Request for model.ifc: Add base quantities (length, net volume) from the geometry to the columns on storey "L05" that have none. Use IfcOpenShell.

First a look at what the model holds.

```python
import ifcopenshell
import ifcopenshell.util.element
import ifcopenshell.util.unit

model = ifcopenshell.open("model.ifc")
print(model.schema)
for unit_type in ("LENGTHUNIT", "AREAUNIT", "VOLUMEUNIT"):
    print(unit_type, ifcopenshell.util.unit.calculate_unit_scale(model, unit_type))
storey = next(s for s in model.by_type("IfcBuildingStorey") if s.Name == "L05")
columns = [e for e in ifcopenshell.util.element.get_decomposition(storey) if e.is_a("IfcColumn")]
for e in sorted(columns, key=lambda e: e.id()):
    print(e.id(), e.is_a(), e.Name, list(ifcopenshell.util.element.get_psets(e, qtos_only=True)), sep=" | ")
```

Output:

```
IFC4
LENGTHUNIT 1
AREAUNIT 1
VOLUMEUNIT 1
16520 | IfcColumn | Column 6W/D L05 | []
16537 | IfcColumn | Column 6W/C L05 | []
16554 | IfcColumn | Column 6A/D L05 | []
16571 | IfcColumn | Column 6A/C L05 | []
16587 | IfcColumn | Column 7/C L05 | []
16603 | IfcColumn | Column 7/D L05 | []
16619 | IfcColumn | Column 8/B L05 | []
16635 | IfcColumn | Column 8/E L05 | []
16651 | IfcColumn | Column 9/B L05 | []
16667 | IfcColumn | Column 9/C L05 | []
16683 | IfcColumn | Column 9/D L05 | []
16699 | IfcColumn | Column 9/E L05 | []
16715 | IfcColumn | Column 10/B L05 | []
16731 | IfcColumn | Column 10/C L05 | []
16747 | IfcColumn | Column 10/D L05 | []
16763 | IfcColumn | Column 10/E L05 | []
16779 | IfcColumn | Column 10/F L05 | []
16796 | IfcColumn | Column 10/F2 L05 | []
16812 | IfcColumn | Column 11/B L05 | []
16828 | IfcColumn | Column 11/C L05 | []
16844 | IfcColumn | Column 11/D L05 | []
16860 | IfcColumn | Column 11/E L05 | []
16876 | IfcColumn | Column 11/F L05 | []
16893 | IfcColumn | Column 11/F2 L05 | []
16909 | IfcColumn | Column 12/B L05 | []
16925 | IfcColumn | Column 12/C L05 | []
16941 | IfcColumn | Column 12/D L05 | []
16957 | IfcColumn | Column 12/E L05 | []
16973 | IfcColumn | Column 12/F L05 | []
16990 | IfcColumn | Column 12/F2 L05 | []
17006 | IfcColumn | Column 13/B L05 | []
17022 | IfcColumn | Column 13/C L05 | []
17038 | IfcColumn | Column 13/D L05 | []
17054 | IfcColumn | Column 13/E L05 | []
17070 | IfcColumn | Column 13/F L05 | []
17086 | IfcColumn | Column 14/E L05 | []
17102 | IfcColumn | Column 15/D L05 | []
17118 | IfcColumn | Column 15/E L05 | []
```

```python
import ifcopenshell
import ifcopenshell.api.pset
import ifcopenshell.geom
import ifcopenshell.util.element
import ifcopenshell.util.shape
import ifcopenshell.util.unit

model = ifcopenshell.open("model.ifc")
unit_scale = ifcopenshell.util.unit.calculate_unit_scale(model)
volume_scale = ifcopenshell.util.unit.calculate_unit_scale(model, "VOLUMEUNIT")
settings = ifcopenshell.geom.settings()

storey = next(s for s in model.by_type("IfcBuildingStorey") if s.Name == "L05")
columns = [e for e in ifcopenshell.util.element.get_decomposition(storey) if e.is_a("IfcColumn")]

for e in sorted(columns, key=lambda e: e.id()):
    if ifcopenshell.util.element.get_psets(e, qtos_only=True, should_inherit=False):
        continue
    # Geometry comes back in metres, in the element's own axes.
    shape = ifcopenshell.geom.create_shape(settings, e)
    values = {
        "Length": ifcopenshell.util.shape.get_z(shape.geometry) / unit_scale,
        "NetVolume": ifcopenshell.util.shape.get_volume(shape.geometry) / volume_scale,
    }
    qto = ifcopenshell.api.pset.add_qto(model, product=e, name="Qto_ColumnBaseQuantities")
    ifcopenshell.api.pset.edit_qto(model, qto=qto, properties=values)
    print(e.id(), {k: round(v, 3) for k, v in values.items()})

model.write("model_edited.ifc")
```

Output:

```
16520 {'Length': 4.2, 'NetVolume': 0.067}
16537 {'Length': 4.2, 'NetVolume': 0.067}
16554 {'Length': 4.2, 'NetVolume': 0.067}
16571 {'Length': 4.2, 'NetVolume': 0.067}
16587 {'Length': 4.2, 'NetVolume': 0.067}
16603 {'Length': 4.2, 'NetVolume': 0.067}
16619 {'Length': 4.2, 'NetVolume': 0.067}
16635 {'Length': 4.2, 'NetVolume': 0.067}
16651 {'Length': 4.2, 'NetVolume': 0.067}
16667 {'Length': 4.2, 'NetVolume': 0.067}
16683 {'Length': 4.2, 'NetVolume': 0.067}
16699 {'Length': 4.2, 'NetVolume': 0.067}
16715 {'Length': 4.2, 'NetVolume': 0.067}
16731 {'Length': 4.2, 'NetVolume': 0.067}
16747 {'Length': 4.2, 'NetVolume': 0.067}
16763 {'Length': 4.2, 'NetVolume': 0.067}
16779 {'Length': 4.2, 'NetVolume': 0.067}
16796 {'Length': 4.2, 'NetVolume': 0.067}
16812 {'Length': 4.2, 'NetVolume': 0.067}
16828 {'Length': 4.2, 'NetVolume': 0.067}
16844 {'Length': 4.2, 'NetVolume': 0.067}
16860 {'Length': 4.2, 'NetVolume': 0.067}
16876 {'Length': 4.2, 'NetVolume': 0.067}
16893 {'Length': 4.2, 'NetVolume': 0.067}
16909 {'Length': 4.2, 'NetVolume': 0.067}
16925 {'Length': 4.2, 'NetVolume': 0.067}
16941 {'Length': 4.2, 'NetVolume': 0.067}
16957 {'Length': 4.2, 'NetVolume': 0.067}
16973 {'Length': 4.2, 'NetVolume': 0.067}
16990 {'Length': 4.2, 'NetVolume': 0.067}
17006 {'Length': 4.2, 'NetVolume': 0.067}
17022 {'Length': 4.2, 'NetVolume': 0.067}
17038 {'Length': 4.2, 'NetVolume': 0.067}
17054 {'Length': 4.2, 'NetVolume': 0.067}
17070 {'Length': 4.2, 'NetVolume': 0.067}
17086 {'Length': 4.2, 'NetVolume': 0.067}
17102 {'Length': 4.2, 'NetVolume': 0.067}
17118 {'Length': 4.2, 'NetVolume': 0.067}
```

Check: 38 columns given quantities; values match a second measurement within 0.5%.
